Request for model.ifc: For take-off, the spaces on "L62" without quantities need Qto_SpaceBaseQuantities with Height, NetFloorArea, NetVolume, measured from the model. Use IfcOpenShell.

First a look at what the model holds.

```python
import ifcopenshell
import ifcopenshell.util.element
import ifcopenshell.util.unit

model = ifcopenshell.open("model.ifc")
print(model.schema)
for unit_type in ("LENGTHUNIT", "AREAUNIT", "VOLUMEUNIT"):
    print(unit_type, ifcopenshell.util.unit.calculate_unit_scale(model, unit_type))
storey = next(s for s in model.by_type("IfcBuildingStorey") if s.Name == "L62")
spaces = [e for e in ifcopenshell.util.element.get_decomposition(storey) if e.is_a("IfcSpace")]
for e in sorted(spaces, key=lambda e: e.id()):
    print(e.id(), e.is_a(), e.Name, list(ifcopenshell.util.element.get_psets(e, qtos_only=True)), sep=" | ")
```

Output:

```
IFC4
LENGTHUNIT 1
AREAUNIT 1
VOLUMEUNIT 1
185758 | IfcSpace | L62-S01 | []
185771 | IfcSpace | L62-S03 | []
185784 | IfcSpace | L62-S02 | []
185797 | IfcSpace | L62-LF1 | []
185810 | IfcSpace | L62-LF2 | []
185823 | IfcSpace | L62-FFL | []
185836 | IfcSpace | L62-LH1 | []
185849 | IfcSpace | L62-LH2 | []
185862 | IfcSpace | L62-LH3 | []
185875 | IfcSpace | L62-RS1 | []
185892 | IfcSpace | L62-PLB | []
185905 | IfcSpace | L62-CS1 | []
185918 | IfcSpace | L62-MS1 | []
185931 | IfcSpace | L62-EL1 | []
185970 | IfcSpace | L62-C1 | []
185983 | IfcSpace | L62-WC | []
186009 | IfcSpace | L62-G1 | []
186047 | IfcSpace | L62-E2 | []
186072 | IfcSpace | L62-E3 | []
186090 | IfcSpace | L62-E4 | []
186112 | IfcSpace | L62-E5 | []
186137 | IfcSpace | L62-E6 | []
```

```python
import ifcopenshell
import ifcopenshell.api.pset
import ifcopenshell.geom
import ifcopenshell.util.element
import ifcopenshell.util.shape
import ifcopenshell.util.unit

model = ifcopenshell.open("model.ifc")
unit_scale = ifcopenshell.util.unit.calculate_unit_scale(model)
area_scale = ifcopenshell.util.unit.calculate_unit_scale(model, "AREAUNIT")
volume_scale = ifcopenshell.util.unit.calculate_unit_scale(model, "VOLUMEUNIT")
settings = ifcopenshell.geom.settings()

storey = next(s for s in model.by_type("IfcBuildingStorey") if s.Name == "L62")
spaces = [e for e in ifcopenshell.util.element.get_decomposition(storey) if e.is_a("IfcSpace")]

for e in sorted(spaces, key=lambda e: e.id()):
    if ifcopenshell.util.element.get_psets(e, qtos_only=True, should_inherit=False):
        continue
    # Geometry comes back in metres, in the element's own axes.
    shape = ifcopenshell.geom.create_shape(settings, e)
    values = {
        "Height": ifcopenshell.util.shape.get_z(shape.geometry) / unit_scale,
        "NetFloorArea": ifcopenshell.util.shape.get_footprint_area(shape.geometry) / area_scale,
        "NetVolume": ifcopenshell.util.shape.get_volume(shape.geometry) / volume_scale,
    }
    qto = ifcopenshell.api.pset.add_qto(model, product=e, name="Qto_SpaceBaseQuantities")
    ifcopenshell.api.pset.edit_qto(model, qto=qto, properties=values)
    print(e.id(), {k: round(v, 3) for k, v in values.items()})

model.write("model_edited.ifc")
```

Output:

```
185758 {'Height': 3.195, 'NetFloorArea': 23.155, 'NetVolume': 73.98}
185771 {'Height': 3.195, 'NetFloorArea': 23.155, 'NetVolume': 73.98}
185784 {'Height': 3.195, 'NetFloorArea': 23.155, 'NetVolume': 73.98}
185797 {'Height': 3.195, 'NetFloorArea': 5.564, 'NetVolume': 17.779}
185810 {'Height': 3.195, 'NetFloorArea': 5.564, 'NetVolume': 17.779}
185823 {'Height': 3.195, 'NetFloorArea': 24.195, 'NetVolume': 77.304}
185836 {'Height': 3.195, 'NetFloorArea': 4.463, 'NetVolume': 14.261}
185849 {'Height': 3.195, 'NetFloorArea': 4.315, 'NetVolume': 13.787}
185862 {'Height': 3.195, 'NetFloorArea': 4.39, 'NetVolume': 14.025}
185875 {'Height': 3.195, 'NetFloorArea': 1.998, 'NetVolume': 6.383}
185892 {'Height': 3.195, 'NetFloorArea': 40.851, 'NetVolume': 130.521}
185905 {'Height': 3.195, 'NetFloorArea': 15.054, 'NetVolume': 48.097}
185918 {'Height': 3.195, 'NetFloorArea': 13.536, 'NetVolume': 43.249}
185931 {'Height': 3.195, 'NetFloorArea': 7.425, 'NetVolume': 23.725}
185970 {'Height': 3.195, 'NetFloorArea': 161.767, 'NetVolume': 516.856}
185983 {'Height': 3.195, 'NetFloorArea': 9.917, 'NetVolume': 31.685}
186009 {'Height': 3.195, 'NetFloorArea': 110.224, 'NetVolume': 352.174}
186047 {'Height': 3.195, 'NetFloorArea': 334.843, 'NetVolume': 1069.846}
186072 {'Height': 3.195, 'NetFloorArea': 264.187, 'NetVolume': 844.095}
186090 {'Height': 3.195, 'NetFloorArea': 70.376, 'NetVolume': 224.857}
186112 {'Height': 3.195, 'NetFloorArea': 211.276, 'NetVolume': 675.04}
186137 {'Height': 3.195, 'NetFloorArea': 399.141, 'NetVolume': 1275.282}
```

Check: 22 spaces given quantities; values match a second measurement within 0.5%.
